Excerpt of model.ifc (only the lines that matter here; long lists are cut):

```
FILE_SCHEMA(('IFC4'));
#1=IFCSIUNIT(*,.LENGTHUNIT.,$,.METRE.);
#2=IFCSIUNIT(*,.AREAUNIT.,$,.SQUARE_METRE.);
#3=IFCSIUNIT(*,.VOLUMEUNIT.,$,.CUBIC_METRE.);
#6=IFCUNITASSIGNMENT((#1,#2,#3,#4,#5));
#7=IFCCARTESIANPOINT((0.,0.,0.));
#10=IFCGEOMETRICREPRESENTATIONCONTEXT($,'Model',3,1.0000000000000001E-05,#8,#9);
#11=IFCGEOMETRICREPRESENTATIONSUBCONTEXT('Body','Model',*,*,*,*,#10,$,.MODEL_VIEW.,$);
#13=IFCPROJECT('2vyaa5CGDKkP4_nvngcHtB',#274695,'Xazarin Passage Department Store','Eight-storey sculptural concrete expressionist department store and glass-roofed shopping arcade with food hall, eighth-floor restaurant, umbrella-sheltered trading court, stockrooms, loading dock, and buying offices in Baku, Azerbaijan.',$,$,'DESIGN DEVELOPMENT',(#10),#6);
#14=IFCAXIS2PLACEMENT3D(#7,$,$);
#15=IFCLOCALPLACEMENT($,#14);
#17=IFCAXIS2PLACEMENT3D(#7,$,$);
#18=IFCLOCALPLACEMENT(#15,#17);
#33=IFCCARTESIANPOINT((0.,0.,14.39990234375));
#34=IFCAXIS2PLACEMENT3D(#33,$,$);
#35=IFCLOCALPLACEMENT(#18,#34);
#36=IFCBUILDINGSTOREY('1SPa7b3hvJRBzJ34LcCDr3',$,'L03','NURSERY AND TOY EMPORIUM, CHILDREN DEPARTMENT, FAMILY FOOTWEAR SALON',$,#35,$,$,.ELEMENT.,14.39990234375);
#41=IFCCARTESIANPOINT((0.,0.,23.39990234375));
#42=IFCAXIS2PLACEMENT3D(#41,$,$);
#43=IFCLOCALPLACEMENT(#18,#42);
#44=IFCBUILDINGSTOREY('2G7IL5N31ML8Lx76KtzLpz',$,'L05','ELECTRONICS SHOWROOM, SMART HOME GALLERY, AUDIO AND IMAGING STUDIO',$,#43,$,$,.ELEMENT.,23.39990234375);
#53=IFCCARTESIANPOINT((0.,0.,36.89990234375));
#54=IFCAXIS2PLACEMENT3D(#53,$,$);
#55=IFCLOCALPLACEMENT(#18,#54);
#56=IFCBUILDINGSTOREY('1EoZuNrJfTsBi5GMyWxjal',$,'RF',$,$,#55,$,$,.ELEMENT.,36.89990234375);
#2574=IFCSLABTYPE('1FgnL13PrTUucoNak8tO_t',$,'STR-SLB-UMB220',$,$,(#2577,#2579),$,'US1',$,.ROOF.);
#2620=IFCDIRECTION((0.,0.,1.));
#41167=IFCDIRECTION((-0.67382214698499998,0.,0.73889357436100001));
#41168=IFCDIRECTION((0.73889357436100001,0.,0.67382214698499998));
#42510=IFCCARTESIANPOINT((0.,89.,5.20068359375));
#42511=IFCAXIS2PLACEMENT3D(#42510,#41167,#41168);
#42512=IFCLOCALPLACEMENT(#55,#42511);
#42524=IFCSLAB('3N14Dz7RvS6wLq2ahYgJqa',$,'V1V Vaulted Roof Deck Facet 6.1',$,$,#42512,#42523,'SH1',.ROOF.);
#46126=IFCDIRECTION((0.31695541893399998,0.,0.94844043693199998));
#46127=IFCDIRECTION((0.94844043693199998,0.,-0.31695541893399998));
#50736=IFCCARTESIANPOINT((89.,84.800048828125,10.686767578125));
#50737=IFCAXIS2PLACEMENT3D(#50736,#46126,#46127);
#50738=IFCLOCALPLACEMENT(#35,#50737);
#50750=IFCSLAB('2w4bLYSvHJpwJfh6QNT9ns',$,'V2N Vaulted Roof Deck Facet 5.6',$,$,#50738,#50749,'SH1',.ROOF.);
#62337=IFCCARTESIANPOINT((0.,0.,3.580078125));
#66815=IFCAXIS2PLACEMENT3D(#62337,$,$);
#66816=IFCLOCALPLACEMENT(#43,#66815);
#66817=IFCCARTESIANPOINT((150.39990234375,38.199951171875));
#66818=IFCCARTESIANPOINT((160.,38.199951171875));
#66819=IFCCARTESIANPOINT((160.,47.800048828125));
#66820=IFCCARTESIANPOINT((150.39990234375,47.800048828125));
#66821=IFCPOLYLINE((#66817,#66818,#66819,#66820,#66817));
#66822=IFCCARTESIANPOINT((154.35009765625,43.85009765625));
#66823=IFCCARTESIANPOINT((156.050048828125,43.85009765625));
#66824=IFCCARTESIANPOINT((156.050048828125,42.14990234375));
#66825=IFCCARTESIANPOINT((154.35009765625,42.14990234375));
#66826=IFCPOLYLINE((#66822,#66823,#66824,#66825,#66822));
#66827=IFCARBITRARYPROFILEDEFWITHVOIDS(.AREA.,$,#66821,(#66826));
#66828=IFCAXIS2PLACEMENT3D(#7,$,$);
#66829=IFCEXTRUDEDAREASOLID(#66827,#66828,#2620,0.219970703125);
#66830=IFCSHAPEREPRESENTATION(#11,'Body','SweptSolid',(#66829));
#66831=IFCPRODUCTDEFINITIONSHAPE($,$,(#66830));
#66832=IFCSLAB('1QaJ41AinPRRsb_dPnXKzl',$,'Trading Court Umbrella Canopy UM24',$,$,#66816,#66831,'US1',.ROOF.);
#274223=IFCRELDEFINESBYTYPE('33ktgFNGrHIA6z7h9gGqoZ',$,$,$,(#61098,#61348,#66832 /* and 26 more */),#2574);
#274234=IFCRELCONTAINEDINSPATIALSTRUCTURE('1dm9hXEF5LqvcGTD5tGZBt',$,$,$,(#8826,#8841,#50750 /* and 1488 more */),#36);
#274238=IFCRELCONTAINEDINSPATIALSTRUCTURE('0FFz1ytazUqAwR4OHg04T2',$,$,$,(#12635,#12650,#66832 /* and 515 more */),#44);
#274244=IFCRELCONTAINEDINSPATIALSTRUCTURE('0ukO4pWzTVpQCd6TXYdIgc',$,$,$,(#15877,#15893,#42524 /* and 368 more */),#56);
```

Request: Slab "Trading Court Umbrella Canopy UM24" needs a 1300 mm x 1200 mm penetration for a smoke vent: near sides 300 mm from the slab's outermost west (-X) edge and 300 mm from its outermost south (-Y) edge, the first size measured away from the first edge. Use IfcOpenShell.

```python
import numpy as np
import ifcopenshell
import ifcopenshell.api.feature
import ifcopenshell.api.geometry
import ifcopenshell.api.root
import ifcopenshell.geom
import ifcopenshell.util.placement
import ifcopenshell.util.representation
import ifcopenshell.util.shape
import ifcopenshell.util.unit

model = ifcopenshell.open("model.ifc")
unit_scale = ifcopenshell.util.unit.calculate_unit_scale(model)
settings = ifcopenshell.geom.settings()


def volume(element):
    """Net volume in cubic metres, openings subtracted."""
    shape = ifcopenshell.geom.create_shape(settings, element)
    return ifcopenshell.util.shape.get_volume(shape.geometry)


slab = model.by_id(66832)
before = volume(slab)

# Extent in the slab's own axes, in metres. The edges named are its -X and -Y sides.
slab_shape = ifcopenshell.geom.create_shape(settings, slab)
vertices = ifcopenshell.util.shape.get_vertices(slab_shape.geometry)
x_min, y_min, bottom = vertices.min(axis=0)
top = vertices[:, 2].max()

opening = ifcopenshell.api.root.create_entity(model, ifc_class="IfcOpeningElement", name="Smoke vent opening", predefined_type="OPENING")
context = ifcopenshell.util.representation.get_context(model, "Model", "Body", "MODEL_VIEW")
width, depth = 1.3, 1.2
outline = [(0.0, 0.0), (width, 0.0), (width, depth), (0.0, depth), (0.0, 0.0)]
# Overshoot both faces by 50 mm so the cut is clean.
shape = ifcopenshell.api.geometry.add_slab_representation(
    model, context=context, depth=top - bottom + 0.1, polyline=outline
)
ifcopenshell.api.geometry.assign_representation(model, product=opening, representation=shape)

matrix = ifcopenshell.util.placement.get_local_placement(slab.ObjectPlacement)
matrix[:, 3] = matrix @ np.append(np.array([x_min + 0.3, y_min + 0.3, bottom - 0.05]) / unit_scale, 1.0)
ifcopenshell.api.geometry.edit_object_placement(model, product=opening, matrix=matrix, is_si=False)
ifcopenshell.api.feature.add_feature(model, feature=opening, element=slab)

after = volume(slab)

print(f"slab volume {before:.3f} -> {after:.3f} m3")

model.write("model_rev.ifc")
```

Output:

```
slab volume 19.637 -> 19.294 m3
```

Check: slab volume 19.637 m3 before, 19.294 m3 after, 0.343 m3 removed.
